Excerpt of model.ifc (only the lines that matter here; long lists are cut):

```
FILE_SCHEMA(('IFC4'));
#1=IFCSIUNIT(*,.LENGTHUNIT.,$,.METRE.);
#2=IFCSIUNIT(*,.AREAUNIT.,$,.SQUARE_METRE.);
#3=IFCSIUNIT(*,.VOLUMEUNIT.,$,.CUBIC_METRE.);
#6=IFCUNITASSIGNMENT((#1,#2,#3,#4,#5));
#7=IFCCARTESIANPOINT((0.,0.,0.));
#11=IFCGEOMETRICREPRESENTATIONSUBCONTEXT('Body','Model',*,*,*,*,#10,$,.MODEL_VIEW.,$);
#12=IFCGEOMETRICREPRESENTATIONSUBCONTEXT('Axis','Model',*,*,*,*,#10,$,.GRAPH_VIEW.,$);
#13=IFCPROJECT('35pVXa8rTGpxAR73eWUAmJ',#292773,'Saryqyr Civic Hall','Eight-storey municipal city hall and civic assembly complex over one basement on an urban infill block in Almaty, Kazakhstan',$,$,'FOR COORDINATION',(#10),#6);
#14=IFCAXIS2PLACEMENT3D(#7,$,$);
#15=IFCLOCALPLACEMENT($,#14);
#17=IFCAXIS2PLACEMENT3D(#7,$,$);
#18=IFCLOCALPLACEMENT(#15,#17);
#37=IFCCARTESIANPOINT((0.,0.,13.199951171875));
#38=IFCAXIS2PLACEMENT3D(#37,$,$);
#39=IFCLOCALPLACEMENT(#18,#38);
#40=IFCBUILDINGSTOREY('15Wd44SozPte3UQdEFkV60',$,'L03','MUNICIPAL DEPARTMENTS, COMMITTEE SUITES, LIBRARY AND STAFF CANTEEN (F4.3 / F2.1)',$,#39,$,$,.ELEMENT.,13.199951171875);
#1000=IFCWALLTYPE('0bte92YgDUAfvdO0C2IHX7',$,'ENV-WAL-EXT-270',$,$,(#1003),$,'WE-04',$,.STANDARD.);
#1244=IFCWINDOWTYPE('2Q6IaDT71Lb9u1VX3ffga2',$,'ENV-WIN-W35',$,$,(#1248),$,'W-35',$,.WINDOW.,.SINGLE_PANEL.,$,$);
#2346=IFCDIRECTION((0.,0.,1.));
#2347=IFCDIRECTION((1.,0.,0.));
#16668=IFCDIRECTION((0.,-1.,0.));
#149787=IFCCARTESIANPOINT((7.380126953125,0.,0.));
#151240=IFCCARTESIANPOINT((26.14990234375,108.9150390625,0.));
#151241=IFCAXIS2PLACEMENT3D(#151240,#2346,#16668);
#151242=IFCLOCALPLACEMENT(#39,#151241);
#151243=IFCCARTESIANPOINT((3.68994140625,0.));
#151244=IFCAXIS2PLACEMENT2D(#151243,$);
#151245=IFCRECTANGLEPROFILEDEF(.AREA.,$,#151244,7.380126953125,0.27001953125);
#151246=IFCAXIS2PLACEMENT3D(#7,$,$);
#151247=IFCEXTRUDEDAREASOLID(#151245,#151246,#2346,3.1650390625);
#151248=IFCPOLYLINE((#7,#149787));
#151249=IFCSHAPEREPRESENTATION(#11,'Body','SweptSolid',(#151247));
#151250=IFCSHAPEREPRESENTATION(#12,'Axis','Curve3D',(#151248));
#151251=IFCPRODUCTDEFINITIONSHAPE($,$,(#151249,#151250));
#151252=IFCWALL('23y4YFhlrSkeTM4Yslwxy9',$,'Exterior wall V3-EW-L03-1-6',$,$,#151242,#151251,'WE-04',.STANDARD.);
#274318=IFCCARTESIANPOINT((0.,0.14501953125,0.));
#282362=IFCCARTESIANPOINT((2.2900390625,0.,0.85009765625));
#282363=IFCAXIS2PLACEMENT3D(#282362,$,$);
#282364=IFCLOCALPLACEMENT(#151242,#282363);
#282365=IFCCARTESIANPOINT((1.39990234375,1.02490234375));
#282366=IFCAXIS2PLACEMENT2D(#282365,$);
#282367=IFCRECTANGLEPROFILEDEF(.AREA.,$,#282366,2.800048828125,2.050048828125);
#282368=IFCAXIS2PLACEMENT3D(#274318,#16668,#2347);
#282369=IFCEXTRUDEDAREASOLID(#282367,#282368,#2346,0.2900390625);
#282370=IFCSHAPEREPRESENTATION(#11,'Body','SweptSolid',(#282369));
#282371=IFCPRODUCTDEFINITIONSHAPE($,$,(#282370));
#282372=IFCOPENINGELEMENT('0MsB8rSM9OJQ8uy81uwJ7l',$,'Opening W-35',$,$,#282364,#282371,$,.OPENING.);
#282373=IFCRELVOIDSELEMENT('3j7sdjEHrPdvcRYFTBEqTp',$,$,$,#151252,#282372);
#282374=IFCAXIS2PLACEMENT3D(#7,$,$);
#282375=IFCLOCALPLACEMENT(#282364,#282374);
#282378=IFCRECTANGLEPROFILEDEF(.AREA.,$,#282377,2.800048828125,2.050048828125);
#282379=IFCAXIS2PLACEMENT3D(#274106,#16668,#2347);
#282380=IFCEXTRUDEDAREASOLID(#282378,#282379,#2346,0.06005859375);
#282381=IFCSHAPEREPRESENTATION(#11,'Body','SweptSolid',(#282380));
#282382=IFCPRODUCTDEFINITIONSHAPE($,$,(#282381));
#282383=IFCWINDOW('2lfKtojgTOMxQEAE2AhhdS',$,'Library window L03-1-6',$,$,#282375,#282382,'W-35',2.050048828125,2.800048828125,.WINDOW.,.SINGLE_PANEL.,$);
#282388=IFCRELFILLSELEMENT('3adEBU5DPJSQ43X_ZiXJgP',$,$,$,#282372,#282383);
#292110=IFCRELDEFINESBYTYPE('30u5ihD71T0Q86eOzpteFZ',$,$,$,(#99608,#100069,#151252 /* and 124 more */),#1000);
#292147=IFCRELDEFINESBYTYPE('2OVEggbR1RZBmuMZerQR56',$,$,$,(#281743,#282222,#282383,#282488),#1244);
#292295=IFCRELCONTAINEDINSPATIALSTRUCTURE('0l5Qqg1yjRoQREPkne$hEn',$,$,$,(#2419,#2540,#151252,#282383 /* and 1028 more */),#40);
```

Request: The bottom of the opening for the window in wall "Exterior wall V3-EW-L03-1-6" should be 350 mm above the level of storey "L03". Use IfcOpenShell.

```python
import numpy as np
import ifcopenshell
import ifcopenshell.api.geometry
import ifcopenshell.geom
import ifcopenshell.util.element
import ifcopenshell.util.placement
import ifcopenshell.util.shape
import ifcopenshell.util.unit

model = ifcopenshell.open("model.ifc")
unit_scale = ifcopenshell.util.unit.calculate_unit_scale(model)

window = model.by_guid("2lfKtojgTOMxQEAE2AhhdS")
opening = window.FillsVoids[0].RelatingOpeningElement
storey = ifcopenshell.util.element.get_container(window, ifc_class="IfcBuildingStorey")
level = ifcopenshell.util.placement.get_local_placement(storey.ObjectPlacement)[2, 3]

# The opening's origin need not be at the sill, so measure its lowest point.
shape = ifcopenshell.geom.create_shape(ifcopenshell.geom.settings(), opening)
bottom = ifcopenshell.util.shape.get_shape_bottom_elevation(shape, shape.geometry) / unit_scale
dz = level + 0.35 / unit_scale - bottom

shift = np.array([0.0, 0.0, dz])
# The window is placed relative to its opening, so it follows when the opening moves.
matrix = ifcopenshell.util.placement.get_local_placement(opening.ObjectPlacement)
matrix[:3, 3] += shift
ifcopenshell.api.geometry.edit_object_placement(
    model, product=opening, matrix=matrix, is_si=False, should_transform_children=True
)

print(f"moved by {dz * unit_scale:+.3f} m")

model.write("model_v2.ifc")
```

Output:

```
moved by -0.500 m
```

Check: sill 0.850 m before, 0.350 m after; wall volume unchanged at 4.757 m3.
